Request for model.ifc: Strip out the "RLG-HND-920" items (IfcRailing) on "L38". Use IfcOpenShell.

First a look at what the model holds.

```python
import ifcopenshell
import ifcopenshell.util.element

model = ifcopenshell.open("model.ifc")
print(model.schema)
storey = next(s for s in model.by_type("IfcBuildingStorey") if s.Name == "L38")
railings = [e for e in ifcopenshell.util.element.get_decomposition(storey) if e.is_a("IfcRailing")]
seen = {}
for e in railings:
    element_type = ifcopenshell.util.element.get_type(e)
    name = element_type.Name if element_type not in (None, e) else None
    seen[name] = seen.get(name, 0) + 1
for name, count in sorted(seen.items(), key=str):
    print(count, "x", name)
```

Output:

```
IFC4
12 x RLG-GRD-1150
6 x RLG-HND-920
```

```python
import ifcopenshell
import ifcopenshell.api.root
import ifcopenshell.util.element

model = ifcopenshell.open("model.ifc")

storey = next(s for s in model.by_type("IfcBuildingStorey") if s.Name == "L38")
railings = [e for e in ifcopenshell.util.element.get_decomposition(storey) if e.is_a("IfcRailing")]
targets = [e for e in railings if (t := ifcopenshell.util.element.get_type(e)) not in (None, e) and t.Name == "RLG-HND-920"]

for e in targets:
    ifcopenshell.api.root.remove_product(model, product=e)
print(len(targets), "removed")

model.write("model-out.ifc")
```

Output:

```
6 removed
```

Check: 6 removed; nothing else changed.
